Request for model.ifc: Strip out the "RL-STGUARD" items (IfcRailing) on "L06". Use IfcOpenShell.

First a look at what the model holds.

```python
import ifcopenshell
import ifcopenshell.util.element

model = ifcopenshell.open("model.ifc")
print(model.schema)
storey = next(s for s in model.by_type("IfcBuildingStorey") if s.Name == "L06")
railings = [e for e in ifcopenshell.util.element.get_decomposition(storey) if e.is_a("IfcRailing")]
seen = {}
for e in railings:
    element_type = ifcopenshell.util.element.get_type(e)
    name = element_type.Name if element_type not in (None, e) else None
    seen[name] = seen.get(name, 0) + 1
for name, count in sorted(seen.items(), key=str):
    print(count, "x", name)
```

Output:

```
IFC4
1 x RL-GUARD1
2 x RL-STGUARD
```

```python
import ifcopenshell
import ifcopenshell.api.root
import ifcopenshell.util.element

model = ifcopenshell.open("model.ifc")

storey = next(s for s in model.by_type("IfcBuildingStorey") if s.Name == "L06")
railings = [e for e in ifcopenshell.util.element.get_decomposition(storey) if e.is_a("IfcRailing")]
targets = [e for e in railings if (t := ifcopenshell.util.element.get_type(e)) not in (None, e) and t.Name == "RL-STGUARD"]

for e in targets:
    ifcopenshell.api.root.remove_product(model, product=e)
print(len(targets), "removed")

model.write("model_rev.ifc")
```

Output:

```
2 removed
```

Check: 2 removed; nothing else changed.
